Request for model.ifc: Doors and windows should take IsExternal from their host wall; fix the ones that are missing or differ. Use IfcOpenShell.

First a look at what the model holds.

```python
import ifcopenshell
import ifcopenshell.util.element

model = ifcopenshell.open("model.ifc")
print(model.schema)
seen = {}
for e in model.by_type("IfcDoor") + model.by_type("IfcWindow"):
    if not e.FillsVoids:
        continue
    host = e.FillsVoids[0].RelatingOpeningElement.VoidsElements[0].RelatingBuildingElement
    own = ifcopenshell.util.element.get_pset(e, f"Pset_{e.is_a()[3:].removesuffix('StandardCase')}Common", "IsExternal")
    wall = ifcopenshell.util.element.get_pset(host, "Pset_WallCommon", "IsExternal")
    seen[e.is_a(), own, wall] = seen.get((e.is_a(), own, wall), 0) + 1
for (cls, own, wall), count in sorted(seen.items(), key=str):
    print(count, cls, "IsExternal:", own, "| host wall:", wall)
```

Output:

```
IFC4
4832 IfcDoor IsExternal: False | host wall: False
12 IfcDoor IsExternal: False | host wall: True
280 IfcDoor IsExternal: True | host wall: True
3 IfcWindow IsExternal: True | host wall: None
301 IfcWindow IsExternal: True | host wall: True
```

```python
import ifcopenshell
import ifcopenshell.api.pset
import ifcopenshell.util.element

model = ifcopenshell.open("model.ifc")

count = 0
for ifc_class, pset_name in (("IfcDoor", "Pset_DoorCommon"), ("IfcWindow", "Pset_WindowCommon")):
    for e in model.by_type(ifc_class):
        if not e.FillsVoids:
            continue
        host = e.FillsVoids[0].RelatingOpeningElement.VoidsElements[0].RelatingBuildingElement
        external = ifcopenshell.util.element.get_pset(host, "Pset_WallCommon", "IsExternal")
        if external is None or ifcopenshell.util.element.get_pset(e, pset_name, "IsExternal") == external:
            continue
        pset = ifcopenshell.api.pset.add_pset(model, product=e, name=pset_name)
        ifcopenshell.api.pset.edit_pset(model, pset=pset, properties={"IsExternal": external})
        count += 1

print(count, "updated")

model.write("model_rev.ifc")
```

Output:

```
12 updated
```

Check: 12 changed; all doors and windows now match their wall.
